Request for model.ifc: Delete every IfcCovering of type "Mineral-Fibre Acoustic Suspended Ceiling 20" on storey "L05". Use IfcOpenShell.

First a look at what the model holds.

```python
import ifcopenshell
import ifcopenshell.util.element

model = ifcopenshell.open("model.ifc")
print(model.schema)
storey = next(s for s in model.by_type("IfcBuildingStorey") if s.Name == "L05")
coverings = [e for e in ifcopenshell.util.element.get_decomposition(storey) if e.is_a("IfcCovering")]
seen = {}
for e in coverings:
    element_type = ifcopenshell.util.element.get_type(e)
    name = element_type.Name if element_type not in (None, e) else None
    seen[name] = seen.get(name, 0) + 1
for name, count in sorted(seen.items(), key=str):
    print(count, "x", name)
```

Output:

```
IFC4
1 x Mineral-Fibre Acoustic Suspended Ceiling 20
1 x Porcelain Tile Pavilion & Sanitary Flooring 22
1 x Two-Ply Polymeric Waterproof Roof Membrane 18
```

```python
import ifcopenshell
import ifcopenshell.api.root
import ifcopenshell.util.element

model = ifcopenshell.open("model.ifc")

storey = next(s for s in model.by_type("IfcBuildingStorey") if s.Name == "L05")
coverings = [e for e in ifcopenshell.util.element.get_decomposition(storey) if e.is_a("IfcCovering")]
targets = [e for e in coverings if (t := ifcopenshell.util.element.get_type(e)) not in (None, e) and t.Name == "Mineral-Fibre Acoustic Suspended Ceiling 20"]

for e in targets:
    ifcopenshell.api.root.remove_product(model, product=e)
print(len(targets), "removed")

model.write("model_v2.ifc")
```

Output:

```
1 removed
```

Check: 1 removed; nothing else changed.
